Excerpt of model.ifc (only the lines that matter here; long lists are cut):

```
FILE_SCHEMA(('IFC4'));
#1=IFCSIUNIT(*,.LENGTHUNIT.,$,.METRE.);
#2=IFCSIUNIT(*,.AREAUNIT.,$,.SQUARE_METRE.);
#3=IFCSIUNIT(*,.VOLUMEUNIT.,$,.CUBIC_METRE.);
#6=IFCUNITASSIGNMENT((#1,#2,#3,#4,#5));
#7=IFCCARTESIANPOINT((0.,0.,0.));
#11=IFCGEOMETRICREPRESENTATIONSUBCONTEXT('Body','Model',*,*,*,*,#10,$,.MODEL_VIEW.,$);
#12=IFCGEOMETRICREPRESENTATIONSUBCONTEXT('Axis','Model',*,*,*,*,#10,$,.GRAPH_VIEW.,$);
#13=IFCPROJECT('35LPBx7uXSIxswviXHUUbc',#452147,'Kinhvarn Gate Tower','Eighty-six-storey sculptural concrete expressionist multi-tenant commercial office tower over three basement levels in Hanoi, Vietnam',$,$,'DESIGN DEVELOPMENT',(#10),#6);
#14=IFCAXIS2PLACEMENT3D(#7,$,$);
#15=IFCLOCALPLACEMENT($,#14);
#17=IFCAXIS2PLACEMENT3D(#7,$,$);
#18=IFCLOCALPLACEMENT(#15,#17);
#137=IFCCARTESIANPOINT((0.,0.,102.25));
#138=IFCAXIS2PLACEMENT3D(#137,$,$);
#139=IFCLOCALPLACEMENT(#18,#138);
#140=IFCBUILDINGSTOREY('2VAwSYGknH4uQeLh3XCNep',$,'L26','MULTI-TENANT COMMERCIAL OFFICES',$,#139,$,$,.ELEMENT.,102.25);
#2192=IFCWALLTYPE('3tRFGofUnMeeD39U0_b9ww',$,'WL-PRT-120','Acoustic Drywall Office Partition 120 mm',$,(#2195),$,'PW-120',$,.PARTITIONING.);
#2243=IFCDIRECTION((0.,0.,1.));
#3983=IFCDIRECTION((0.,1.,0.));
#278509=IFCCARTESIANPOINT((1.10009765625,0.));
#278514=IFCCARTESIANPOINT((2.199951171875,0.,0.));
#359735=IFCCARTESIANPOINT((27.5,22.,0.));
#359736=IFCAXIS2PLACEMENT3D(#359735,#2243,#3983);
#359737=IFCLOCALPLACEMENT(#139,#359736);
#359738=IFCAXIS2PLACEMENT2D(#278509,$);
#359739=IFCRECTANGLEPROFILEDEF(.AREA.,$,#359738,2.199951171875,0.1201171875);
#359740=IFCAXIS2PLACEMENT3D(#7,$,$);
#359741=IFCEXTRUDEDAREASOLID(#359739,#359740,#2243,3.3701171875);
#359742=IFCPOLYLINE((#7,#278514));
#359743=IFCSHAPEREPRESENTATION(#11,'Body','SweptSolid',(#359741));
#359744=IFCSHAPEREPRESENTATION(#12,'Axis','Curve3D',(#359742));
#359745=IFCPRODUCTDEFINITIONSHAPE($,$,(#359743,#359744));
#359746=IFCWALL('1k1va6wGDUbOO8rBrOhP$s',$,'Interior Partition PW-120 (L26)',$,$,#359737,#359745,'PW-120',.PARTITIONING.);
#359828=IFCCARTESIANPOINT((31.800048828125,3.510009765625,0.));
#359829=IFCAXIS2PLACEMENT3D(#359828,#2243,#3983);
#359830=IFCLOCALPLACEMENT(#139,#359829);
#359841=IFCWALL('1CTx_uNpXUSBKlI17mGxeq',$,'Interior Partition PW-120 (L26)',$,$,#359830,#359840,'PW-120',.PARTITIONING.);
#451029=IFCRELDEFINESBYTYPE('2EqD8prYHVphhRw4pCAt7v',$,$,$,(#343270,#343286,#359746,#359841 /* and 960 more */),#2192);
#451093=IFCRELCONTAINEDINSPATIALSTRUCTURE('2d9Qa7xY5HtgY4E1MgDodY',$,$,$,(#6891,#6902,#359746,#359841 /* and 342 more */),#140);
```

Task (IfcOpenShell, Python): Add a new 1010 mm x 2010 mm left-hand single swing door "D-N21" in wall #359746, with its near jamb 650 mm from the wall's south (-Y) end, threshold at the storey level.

```python
import numpy as np
import ifcopenshell
import ifcopenshell.api.feature
import ifcopenshell.api.geometry
import ifcopenshell.api.root
import ifcopenshell.api.spatial
import ifcopenshell.geom
import ifcopenshell.util.element
import ifcopenshell.util.placement
import ifcopenshell.util.representation
import ifcopenshell.util.shape
import ifcopenshell.util.unit

model = ifcopenshell.open("model.ifc")
unit_scale = ifcopenshell.util.unit.calculate_unit_scale(model)
settings = ifcopenshell.geom.settings()


def volume(element):
    """Net volume in cubic metres, openings subtracted."""
    shape = ifcopenshell.geom.create_shape(settings, element)
    return ifcopenshell.util.shape.get_volume(shape.geometry)


wall = model.by_id(359746)
storey = ifcopenshell.util.element.get_container(wall, ifc_class="IfcBuildingStorey")
context = ifcopenshell.util.representation.get_context(model, "Model", "Body", "MODEL_VIEW")
before = volume(wall)

width, height, from_end, sill = 1.01, 2.01, 0.65, 0.0  # metres

# The wall runs along its own X axis, and the end named is its -X end.
wall_shape = ifcopenshell.geom.create_shape(settings, wall)
x, y, z = ifcopenshell.util.shape.get_vertices(wall_shape.geometry).T
start = x.min() + from_end
face, thickness = float(y.min()), float(y.max() - y.min())
wall_matrix = ifcopenshell.util.placement.get_local_placement(wall.ObjectPlacement)
level = ifcopenshell.util.placement.get_local_placement(storey.ObjectPlacement)[2, 3]


def in_wall(x, y):
    """Placement at x, y metres in the wall's axes, at sill height."""
    matrix = wall_matrix.copy()
    matrix[:, 3] = wall_matrix @ np.array([x / unit_scale, y / unit_scale, 0.0, 1.0])
    matrix[2, 3] = level + sill / unit_scale
    return matrix


# Opening: a box that overshoots both wall faces by 50 mm.
opening = ifcopenshell.api.root.create_entity(model, ifc_class="IfcOpeningElement", predefined_type="OPENING")
box = ifcopenshell.api.geometry.add_wall_representation(
    model, context=context, length=width, height=height, thickness=thickness + 0.1
)
ifcopenshell.api.geometry.assign_representation(model, product=opening, representation=box)
ifcopenshell.api.geometry.edit_object_placement(model, product=opening, matrix=in_wall(start, face - 0.05), is_si=False)
ifcopenshell.api.feature.add_feature(model, feature=opening, element=wall)

door = ifcopenshell.api.root.create_entity(model, ifc_class="IfcDoor", name="D-N21", predefined_type="DOOR")
door.OverallWidth, door.OverallHeight = width / unit_scale, height / unit_scale
door.OperationType = "SINGLE_SWING_LEFT"
body = ifcopenshell.api.geometry.add_door_representation(
    model,
    context=context,
    overall_width=door.OverallWidth,
    overall_height=door.OverallHeight,
    operation_type="SINGLE_SWING_LEFT",
    lining_properties={"LiningDepth": thickness / unit_scale, "ThresholdDepth": thickness / unit_scale},
)
ifcopenshell.api.geometry.assign_representation(model, product=door, representation=body)
ifcopenshell.api.spatial.assign_container(model, products=[door], relating_structure=storey)
ifcopenshell.api.feature.add_filling(model, opening=opening, element=door)

# The lining spans the wall, so the door starts at the wall face.
ifcopenshell.api.geometry.edit_object_placement(model, product=door, matrix=in_wall(start, face), is_si=False)

after = volume(wall)

print(f"wall volume {before:.3f} -> {after:.3f} m3")

model.write("model_rev.ifc")
```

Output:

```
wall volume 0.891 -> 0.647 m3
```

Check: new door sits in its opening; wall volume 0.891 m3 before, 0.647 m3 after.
